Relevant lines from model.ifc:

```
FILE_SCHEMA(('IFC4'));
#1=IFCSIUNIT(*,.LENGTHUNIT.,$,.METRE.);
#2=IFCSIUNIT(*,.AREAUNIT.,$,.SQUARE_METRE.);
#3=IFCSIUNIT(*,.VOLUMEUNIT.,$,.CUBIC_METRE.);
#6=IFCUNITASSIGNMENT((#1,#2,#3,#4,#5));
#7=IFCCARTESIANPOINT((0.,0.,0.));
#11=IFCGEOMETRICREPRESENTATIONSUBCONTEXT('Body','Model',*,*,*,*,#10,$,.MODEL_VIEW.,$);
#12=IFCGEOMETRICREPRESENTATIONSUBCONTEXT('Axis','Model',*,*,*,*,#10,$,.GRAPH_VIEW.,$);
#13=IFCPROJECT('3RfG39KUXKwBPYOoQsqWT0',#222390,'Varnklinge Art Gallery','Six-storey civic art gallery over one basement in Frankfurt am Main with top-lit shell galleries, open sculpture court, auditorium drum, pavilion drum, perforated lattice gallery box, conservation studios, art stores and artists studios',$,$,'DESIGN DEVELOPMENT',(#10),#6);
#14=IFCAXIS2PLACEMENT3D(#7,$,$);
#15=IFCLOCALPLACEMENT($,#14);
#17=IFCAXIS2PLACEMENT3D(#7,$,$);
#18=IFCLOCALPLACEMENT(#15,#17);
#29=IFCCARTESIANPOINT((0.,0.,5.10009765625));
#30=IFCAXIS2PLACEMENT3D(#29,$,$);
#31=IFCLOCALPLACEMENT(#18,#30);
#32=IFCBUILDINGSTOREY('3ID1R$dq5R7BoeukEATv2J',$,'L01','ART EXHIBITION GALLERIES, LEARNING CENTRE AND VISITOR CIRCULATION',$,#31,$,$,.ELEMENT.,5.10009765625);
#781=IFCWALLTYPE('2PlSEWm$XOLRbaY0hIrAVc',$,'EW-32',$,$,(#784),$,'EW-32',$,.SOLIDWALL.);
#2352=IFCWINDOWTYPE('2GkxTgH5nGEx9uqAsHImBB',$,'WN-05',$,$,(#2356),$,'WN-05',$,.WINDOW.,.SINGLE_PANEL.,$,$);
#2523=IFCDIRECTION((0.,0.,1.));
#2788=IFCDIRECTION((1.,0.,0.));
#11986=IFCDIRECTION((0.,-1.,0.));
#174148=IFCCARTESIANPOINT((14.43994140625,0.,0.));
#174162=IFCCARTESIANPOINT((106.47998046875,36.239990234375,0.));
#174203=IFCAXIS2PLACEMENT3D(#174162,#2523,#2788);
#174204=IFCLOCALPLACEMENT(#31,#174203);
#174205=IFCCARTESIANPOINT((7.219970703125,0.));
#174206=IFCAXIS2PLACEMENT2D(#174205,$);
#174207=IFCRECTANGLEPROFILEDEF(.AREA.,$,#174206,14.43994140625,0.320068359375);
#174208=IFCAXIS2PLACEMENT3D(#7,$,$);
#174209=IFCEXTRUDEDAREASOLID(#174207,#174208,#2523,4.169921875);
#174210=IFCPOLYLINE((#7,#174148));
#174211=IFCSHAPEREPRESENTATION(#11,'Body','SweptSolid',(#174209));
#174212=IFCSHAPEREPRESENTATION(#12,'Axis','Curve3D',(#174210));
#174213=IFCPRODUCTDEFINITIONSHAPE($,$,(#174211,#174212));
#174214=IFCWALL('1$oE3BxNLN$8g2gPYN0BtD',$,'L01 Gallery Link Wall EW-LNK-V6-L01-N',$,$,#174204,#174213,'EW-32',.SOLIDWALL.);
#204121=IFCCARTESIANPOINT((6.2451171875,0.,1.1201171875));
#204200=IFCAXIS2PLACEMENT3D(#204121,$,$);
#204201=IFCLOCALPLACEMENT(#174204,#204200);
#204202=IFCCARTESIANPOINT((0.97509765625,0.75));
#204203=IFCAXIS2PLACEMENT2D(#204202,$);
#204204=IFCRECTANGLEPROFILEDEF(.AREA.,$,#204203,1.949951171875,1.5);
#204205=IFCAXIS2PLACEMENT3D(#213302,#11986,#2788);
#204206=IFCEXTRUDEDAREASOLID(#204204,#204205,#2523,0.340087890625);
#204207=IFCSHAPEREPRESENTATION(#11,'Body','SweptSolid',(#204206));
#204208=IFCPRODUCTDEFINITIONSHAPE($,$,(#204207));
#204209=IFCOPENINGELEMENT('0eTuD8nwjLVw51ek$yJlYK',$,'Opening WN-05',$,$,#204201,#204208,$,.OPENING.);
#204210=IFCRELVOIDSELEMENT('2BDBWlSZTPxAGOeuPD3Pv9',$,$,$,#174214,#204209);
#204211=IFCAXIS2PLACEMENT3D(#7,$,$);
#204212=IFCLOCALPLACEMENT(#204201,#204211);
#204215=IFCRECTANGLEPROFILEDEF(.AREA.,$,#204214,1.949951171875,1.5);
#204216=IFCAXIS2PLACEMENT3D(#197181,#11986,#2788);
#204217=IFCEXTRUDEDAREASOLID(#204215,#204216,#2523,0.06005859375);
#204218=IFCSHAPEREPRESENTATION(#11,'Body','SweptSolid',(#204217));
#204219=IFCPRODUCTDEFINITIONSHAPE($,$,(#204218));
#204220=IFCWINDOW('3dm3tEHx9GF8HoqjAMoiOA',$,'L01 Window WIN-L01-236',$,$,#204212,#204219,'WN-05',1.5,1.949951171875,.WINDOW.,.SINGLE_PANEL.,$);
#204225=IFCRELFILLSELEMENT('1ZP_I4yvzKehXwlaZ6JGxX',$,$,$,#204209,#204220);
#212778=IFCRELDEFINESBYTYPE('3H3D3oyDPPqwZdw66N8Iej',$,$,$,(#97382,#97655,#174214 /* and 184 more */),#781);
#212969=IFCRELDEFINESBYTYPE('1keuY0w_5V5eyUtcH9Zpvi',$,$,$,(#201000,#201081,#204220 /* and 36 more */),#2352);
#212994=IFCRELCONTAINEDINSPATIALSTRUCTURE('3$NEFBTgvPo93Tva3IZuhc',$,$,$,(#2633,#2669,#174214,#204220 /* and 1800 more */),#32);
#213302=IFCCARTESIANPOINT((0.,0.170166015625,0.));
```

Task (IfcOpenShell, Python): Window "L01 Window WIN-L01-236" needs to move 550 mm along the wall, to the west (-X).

```python
import ifcopenshell
import ifcopenshell.api.geometry
import ifcopenshell.util.placement
import ifcopenshell.util.unit

model = ifcopenshell.open("model.ifc")
unit_scale = ifcopenshell.util.unit.calculate_unit_scale(model)

window = model.by_guid("3dm3tEHx9GF8HoqjAMoiOA")
opening = window.FillsVoids[0].RelatingOpeningElement
wall = opening.VoidsElements[0].RelatingBuildingElement

wall_matrix = ifcopenshell.util.placement.get_local_placement(wall.ObjectPlacement)
shift = wall_matrix[:3, 0] * -0.55 / unit_scale
before = ifcopenshell.util.placement.get_local_placement(window.ObjectPlacement)[:3, 3].copy()

# The window is placed relative to its opening, so it follows when the opening moves.
matrix = ifcopenshell.util.placement.get_local_placement(opening.ObjectPlacement)
matrix[:3, 3] += shift
ifcopenshell.api.geometry.edit_object_placement(
    model, product=opening, matrix=matrix, is_si=False, should_transform_children=True
)

after = ifcopenshell.util.placement.get_local_placement(window.ObjectPlacement)[:3, 3]
print("window moved by", (after - before).round(3) + 0.0)

model.write("model_v2.ifc")
```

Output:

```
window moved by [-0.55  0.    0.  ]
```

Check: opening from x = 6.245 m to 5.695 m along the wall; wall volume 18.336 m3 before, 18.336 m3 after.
